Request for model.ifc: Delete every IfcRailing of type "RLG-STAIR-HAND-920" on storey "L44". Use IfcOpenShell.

First a look at what the model holds.

```python
import ifcopenshell
import ifcopenshell.util.element

model = ifcopenshell.open("model.ifc")
print(model.schema)
storey = next(s for s in model.by_type("IfcBuildingStorey") if s.Name == "L44")
railings = [e for e in ifcopenshell.util.element.get_decomposition(storey) if e.is_a("IfcRailing")]
seen = {}
for e in railings:
    element_type = ifcopenshell.util.element.get_type(e)
    name = element_type.Name if element_type not in (None, e) else None
    seen[name] = seen.get(name, 0) + 1
for name, count in sorted(seen.items(), key=str):
    print(count, "x", name)
```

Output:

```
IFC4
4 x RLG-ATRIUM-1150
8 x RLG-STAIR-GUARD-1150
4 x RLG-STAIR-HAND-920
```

```python
import ifcopenshell
import ifcopenshell.api.root
import ifcopenshell.util.element

model = ifcopenshell.open("model.ifc")

storey = next(s for s in model.by_type("IfcBuildingStorey") if s.Name == "L44")
railings = [e for e in ifcopenshell.util.element.get_decomposition(storey) if e.is_a("IfcRailing")]
targets = [e for e in railings if (t := ifcopenshell.util.element.get_type(e)) not in (None, e) and t.Name == "RLG-STAIR-HAND-920"]

for e in targets:
    ifcopenshell.api.root.remove_product(model, product=e)
print(len(targets), "removed")

model.write("model_v2.ifc")
```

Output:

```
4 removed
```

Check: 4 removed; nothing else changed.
